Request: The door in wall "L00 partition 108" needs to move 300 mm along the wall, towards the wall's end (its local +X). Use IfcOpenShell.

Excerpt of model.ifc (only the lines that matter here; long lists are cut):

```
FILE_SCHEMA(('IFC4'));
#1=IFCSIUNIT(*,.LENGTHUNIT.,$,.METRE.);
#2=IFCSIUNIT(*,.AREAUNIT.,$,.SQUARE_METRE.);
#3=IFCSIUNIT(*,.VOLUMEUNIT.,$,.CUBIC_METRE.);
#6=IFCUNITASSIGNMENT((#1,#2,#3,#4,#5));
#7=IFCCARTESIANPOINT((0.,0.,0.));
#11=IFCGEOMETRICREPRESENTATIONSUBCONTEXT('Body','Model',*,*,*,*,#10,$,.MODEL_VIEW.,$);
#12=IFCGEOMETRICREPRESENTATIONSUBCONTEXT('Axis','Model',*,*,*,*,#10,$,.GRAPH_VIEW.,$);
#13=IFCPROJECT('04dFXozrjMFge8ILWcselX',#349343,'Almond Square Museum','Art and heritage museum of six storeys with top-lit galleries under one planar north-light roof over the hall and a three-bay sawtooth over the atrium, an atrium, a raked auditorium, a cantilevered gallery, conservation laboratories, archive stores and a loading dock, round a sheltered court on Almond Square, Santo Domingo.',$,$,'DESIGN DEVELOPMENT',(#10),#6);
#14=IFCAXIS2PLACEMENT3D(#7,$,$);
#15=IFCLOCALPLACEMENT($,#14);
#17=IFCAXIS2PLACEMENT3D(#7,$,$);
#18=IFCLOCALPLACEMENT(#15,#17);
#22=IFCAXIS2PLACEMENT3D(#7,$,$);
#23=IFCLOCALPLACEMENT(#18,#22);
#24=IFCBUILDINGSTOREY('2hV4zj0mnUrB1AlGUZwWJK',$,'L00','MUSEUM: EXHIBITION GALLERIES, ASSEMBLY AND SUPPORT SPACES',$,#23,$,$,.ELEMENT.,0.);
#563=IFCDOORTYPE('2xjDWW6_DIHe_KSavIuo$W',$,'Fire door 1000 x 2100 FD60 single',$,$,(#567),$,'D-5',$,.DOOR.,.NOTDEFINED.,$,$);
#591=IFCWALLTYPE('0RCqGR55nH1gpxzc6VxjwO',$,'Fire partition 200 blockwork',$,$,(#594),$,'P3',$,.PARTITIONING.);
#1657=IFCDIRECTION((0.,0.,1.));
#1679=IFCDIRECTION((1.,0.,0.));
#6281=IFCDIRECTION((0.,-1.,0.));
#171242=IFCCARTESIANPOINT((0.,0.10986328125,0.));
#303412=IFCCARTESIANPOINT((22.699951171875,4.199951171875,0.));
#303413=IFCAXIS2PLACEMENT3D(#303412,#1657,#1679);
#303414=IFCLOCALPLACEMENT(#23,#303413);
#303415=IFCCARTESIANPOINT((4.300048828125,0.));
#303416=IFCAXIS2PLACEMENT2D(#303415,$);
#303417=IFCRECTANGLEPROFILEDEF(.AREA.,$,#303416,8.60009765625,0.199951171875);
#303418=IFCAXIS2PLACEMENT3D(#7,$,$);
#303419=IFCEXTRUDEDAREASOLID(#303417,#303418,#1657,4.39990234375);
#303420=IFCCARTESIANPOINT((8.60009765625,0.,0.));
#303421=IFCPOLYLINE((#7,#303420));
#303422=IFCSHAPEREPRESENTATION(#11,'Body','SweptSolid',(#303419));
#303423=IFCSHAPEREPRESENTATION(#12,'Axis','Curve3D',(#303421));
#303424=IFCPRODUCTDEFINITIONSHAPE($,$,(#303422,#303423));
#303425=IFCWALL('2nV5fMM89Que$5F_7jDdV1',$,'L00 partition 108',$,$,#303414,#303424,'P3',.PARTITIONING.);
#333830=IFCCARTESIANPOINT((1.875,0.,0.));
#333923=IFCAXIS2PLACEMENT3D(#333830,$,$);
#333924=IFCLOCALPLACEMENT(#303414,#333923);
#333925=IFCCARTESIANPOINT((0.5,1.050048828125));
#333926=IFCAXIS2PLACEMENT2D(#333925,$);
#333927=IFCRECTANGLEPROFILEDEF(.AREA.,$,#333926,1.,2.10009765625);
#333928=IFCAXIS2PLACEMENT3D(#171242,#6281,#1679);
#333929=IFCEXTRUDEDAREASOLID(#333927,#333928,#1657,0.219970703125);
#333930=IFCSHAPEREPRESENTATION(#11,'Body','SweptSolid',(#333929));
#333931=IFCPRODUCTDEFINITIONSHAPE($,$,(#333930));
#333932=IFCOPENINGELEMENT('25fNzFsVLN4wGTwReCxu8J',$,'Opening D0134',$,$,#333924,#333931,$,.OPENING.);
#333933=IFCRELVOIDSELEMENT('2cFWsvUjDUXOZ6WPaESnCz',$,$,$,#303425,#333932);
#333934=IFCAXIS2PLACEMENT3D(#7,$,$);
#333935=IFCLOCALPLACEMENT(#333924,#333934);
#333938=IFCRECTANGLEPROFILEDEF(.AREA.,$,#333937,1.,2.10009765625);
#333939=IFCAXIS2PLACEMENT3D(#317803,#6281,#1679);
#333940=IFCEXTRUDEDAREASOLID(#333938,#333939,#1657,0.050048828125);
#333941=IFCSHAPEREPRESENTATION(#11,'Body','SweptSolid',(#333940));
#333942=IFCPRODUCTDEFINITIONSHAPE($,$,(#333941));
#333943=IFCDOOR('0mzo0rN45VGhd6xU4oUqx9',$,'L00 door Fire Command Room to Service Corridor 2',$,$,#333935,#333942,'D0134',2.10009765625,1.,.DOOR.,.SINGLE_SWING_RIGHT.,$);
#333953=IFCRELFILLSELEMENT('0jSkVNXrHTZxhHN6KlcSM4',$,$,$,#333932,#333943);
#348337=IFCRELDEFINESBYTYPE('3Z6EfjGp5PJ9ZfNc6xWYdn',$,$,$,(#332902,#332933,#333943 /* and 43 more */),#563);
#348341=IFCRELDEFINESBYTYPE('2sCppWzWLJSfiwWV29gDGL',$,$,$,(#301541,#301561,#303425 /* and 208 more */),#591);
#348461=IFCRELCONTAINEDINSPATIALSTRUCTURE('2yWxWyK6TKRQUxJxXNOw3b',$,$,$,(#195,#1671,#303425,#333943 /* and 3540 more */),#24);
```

```python
import ifcopenshell
import ifcopenshell.api.geometry
import ifcopenshell.util.placement
import ifcopenshell.util.unit

model = ifcopenshell.open("model.ifc")
unit_scale = ifcopenshell.util.unit.calculate_unit_scale(model)

door = model.by_id(333943)
opening = door.FillsVoids[0].RelatingOpeningElement
wall = opening.VoidsElements[0].RelatingBuildingElement

wall_matrix = ifcopenshell.util.placement.get_local_placement(wall.ObjectPlacement)
shift = wall_matrix[:3, 0] * 0.3 / unit_scale
before = ifcopenshell.util.placement.get_local_placement(door.ObjectPlacement)[:3, 3].copy()

# The door is placed relative to its opening, so it follows when the opening moves.
matrix = ifcopenshell.util.placement.get_local_placement(opening.ObjectPlacement)
matrix[:3, 3] += shift
ifcopenshell.api.geometry.edit_object_placement(
    model, product=opening, matrix=matrix, is_si=False, should_transform_children=True
)

after = ifcopenshell.util.placement.get_local_placement(door.ObjectPlacement)[:3, 3]
print("door moved by", (after - before).round(3) + 0.0)

model.write("model_v2.ifc")
```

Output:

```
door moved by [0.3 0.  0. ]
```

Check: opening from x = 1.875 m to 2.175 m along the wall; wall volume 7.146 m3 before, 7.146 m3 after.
